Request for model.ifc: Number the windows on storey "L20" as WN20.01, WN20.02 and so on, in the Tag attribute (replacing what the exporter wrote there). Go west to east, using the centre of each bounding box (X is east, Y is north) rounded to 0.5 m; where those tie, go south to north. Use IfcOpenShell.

First a look at what the model holds.

```python
import ifcopenshell
import ifcopenshell.util.element
import ifcopenshell.util.placement

model = ifcopenshell.open("model.ifc")
print(model.schema)
storey = next(s for s in model.by_type("IfcBuildingStorey") if s.Name == "L20")
windows = [e for e in ifcopenshell.util.element.get_decomposition(storey) if e.is_a("IfcWindow")]
for e in sorted(windows, key=lambda e: e.id()):
    origin = ifcopenshell.util.placement.get_local_placement(e.ObjectPlacement)[:3, 3]
    print(e.id(), e.Tag, e.Name, origin.round(2) + 0.0, sep=" | ")
```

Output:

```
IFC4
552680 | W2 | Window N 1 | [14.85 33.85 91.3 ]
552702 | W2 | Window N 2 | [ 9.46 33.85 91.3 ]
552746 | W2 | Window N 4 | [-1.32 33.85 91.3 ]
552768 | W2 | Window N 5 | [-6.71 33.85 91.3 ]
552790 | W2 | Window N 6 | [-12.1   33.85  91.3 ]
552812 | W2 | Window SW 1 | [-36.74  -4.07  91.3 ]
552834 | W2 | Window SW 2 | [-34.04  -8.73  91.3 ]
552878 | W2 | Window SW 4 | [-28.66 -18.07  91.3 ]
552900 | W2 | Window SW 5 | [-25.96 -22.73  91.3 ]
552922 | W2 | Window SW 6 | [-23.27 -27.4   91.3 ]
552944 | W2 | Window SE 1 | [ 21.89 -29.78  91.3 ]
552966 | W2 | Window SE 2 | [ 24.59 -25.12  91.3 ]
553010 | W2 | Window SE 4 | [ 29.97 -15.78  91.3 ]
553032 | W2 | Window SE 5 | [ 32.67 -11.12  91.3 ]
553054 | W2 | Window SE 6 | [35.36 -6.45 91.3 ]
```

```python
import ifcopenshell
import ifcopenshell.geom
import ifcopenshell.util.element
import ifcopenshell.util.shape

model = ifcopenshell.open("model.ifc")
settings = ifcopenshell.geom.settings()
settings.set("use-world-coords", True)


def centre(element):
    shape = ifcopenshell.geom.create_shape(settings, element)
    return ifcopenshell.util.shape.get_bbox_centroid(shape.geometry)


storey = next(s for s in model.by_type("IfcBuildingStorey") if s.Name == "L20")
windows = [e for e in ifcopenshell.util.element.get_decomposition(storey) if e.is_a("IfcWindow")]

# Insertion points can sit at a corner or the storey origin, so sort by the geometry (in metres).
centres = {e: centre(e) for e in windows}
windows.sort(key=lambda e: (round(centres[e][0] / 0.5), centres[e][1]))

for i, e in enumerate(windows, start=1):
    number = f"WN20.{i:02d}"
    e.Tag = number
    print(e.id(), number)

model.write("model-out.ifc")
```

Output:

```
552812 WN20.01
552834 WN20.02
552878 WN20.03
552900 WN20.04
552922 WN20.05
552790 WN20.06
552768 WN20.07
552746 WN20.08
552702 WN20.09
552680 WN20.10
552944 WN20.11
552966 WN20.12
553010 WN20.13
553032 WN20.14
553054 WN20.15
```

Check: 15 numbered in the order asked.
